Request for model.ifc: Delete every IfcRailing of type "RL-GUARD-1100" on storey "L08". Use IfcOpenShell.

First a look at what the model holds.

```python
import ifcopenshell
import ifcopenshell.util.element

model = ifcopenshell.open("model.ifc")
print(model.schema)
storey = next(s for s in model.by_type("IfcBuildingStorey") if s.Name == "L08")
railings = [e for e in ifcopenshell.util.element.get_decomposition(storey) if e.is_a("IfcRailing")]
seen = {}
for e in railings:
    element_type = ifcopenshell.util.element.get_type(e)
    name = element_type.Name if element_type not in (None, e) else None
    seen[name] = seen.get(name, 0) + 1
for name, count in sorted(seen.items(), key=str):
    print(count, "x", name)
```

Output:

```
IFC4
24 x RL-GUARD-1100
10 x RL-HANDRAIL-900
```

```python
import ifcopenshell
import ifcopenshell.api.root
import ifcopenshell.util.element

model = ifcopenshell.open("model.ifc")

storey = next(s for s in model.by_type("IfcBuildingStorey") if s.Name == "L08")
railings = [e for e in ifcopenshell.util.element.get_decomposition(storey) if e.is_a("IfcRailing")]
targets = [e for e in railings if (t := ifcopenshell.util.element.get_type(e)) not in (None, e) and t.Name == "RL-GUARD-1100"]

for e in targets:
    ifcopenshell.api.root.remove_product(model, product=e)
print(len(targets), "removed")

model.write("model_rev.ifc")
```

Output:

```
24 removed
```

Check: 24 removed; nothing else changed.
